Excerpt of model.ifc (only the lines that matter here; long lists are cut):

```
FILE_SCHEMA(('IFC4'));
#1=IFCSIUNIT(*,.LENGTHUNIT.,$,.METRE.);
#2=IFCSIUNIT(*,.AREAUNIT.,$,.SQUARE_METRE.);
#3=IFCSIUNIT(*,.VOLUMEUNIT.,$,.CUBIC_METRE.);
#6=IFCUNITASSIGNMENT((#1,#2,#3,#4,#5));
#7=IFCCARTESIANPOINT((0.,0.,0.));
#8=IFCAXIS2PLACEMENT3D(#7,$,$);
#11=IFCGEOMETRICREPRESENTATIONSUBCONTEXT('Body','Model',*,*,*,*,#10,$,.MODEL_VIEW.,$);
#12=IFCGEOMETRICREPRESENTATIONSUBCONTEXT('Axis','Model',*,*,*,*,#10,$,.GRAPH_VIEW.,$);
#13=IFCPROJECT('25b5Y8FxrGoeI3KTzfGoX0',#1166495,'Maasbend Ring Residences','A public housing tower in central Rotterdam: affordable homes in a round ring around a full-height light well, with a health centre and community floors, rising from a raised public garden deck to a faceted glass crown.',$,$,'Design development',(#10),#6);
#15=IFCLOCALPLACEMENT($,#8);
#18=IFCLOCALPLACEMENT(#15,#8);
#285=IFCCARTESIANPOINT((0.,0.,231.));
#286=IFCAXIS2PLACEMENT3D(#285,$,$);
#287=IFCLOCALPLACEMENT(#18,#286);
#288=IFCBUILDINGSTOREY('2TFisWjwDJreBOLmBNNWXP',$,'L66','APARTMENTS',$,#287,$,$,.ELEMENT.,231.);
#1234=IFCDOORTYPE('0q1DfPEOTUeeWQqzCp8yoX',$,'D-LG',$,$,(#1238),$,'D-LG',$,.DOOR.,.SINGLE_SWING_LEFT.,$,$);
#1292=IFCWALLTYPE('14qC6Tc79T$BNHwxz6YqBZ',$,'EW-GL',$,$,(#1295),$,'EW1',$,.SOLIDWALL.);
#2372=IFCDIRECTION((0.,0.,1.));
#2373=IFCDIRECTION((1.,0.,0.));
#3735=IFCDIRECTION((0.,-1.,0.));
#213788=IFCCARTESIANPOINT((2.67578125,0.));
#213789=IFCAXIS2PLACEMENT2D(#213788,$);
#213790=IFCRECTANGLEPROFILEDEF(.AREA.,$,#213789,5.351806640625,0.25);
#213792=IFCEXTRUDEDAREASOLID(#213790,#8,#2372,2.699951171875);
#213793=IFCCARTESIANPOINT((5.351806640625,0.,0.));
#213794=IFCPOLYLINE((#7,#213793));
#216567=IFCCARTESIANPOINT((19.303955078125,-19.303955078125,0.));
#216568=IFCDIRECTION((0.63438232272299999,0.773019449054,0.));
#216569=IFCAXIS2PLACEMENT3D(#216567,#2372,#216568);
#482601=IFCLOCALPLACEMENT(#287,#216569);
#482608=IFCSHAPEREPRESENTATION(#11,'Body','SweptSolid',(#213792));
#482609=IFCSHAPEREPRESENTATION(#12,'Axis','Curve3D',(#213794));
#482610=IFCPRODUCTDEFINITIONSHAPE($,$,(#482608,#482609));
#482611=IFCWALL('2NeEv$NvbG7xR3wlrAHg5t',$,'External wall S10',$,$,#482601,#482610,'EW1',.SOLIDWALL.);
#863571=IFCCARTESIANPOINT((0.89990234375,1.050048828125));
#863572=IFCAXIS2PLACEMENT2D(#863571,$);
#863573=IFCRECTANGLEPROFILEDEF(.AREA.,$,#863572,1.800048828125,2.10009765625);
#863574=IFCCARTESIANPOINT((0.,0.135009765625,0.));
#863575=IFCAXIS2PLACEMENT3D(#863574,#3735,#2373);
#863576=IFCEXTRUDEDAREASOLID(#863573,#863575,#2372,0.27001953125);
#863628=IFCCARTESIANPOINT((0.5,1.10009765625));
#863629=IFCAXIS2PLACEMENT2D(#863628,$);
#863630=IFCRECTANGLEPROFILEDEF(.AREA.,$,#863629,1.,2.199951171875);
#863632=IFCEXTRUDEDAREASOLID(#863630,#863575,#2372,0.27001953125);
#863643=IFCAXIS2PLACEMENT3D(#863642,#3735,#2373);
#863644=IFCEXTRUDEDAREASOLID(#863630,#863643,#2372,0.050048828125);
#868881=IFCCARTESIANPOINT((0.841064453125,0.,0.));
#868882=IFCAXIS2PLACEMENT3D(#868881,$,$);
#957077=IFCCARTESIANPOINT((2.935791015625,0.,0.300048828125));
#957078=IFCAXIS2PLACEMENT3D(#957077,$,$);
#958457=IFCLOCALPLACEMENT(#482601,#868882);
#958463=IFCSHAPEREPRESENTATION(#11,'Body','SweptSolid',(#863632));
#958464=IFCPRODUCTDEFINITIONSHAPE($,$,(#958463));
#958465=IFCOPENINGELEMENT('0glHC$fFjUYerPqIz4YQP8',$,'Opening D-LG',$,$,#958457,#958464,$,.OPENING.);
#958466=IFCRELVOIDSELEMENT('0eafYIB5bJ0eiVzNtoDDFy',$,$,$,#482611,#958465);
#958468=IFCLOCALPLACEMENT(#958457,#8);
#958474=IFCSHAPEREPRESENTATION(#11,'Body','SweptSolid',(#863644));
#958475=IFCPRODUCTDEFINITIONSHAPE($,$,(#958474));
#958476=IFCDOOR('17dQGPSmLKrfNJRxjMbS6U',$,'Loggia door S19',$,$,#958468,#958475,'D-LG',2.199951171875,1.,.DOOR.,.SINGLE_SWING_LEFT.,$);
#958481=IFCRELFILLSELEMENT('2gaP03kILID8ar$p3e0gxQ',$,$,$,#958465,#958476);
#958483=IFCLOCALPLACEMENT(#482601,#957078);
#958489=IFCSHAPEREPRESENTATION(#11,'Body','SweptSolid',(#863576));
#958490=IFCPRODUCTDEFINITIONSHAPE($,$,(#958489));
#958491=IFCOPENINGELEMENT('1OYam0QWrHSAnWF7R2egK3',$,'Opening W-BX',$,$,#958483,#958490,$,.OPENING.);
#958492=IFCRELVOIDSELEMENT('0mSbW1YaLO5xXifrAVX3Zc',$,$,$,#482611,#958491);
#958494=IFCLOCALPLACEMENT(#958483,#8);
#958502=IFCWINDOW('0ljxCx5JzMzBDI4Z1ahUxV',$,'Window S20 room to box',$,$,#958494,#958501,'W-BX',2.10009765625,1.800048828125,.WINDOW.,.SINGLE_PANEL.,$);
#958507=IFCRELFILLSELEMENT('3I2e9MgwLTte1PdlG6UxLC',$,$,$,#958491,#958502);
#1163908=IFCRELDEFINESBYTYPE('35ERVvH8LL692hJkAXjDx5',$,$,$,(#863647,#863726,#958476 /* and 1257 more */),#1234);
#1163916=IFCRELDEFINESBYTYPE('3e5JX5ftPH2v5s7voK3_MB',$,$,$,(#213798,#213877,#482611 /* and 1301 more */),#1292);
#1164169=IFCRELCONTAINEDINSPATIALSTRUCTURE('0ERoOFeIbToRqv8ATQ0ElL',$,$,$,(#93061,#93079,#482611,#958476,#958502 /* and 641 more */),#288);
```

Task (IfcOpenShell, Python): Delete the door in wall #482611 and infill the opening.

```python
import ifcopenshell
import ifcopenshell.api.feature
import ifcopenshell.api.root
import ifcopenshell.geom
import ifcopenshell.util.shape

model = ifcopenshell.open("model.ifc")
settings = ifcopenshell.geom.settings()


def volume(element):
    """Net volume in cubic metres, openings subtracted."""
    shape = ifcopenshell.geom.create_shape(settings, element)
    return ifcopenshell.util.shape.get_volume(shape.geometry)


door = model.by_guid("17dQGPSmLKrfNJRxjMbS6U")
opening = door.FillsVoids[0].RelatingOpeningElement
wall = opening.VoidsElements[0].RelatingBuildingElement
before = volume(wall)

ifcopenshell.api.root.remove_product(model, product=door)
ifcopenshell.api.feature.remove_feature(model, feature=opening)

after = volume(wall)

print(f"wall volume {before:.3f} -> {after:.3f} m3")

model.write("model_edited.ifc")
```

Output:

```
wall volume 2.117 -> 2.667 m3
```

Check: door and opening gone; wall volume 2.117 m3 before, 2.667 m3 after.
